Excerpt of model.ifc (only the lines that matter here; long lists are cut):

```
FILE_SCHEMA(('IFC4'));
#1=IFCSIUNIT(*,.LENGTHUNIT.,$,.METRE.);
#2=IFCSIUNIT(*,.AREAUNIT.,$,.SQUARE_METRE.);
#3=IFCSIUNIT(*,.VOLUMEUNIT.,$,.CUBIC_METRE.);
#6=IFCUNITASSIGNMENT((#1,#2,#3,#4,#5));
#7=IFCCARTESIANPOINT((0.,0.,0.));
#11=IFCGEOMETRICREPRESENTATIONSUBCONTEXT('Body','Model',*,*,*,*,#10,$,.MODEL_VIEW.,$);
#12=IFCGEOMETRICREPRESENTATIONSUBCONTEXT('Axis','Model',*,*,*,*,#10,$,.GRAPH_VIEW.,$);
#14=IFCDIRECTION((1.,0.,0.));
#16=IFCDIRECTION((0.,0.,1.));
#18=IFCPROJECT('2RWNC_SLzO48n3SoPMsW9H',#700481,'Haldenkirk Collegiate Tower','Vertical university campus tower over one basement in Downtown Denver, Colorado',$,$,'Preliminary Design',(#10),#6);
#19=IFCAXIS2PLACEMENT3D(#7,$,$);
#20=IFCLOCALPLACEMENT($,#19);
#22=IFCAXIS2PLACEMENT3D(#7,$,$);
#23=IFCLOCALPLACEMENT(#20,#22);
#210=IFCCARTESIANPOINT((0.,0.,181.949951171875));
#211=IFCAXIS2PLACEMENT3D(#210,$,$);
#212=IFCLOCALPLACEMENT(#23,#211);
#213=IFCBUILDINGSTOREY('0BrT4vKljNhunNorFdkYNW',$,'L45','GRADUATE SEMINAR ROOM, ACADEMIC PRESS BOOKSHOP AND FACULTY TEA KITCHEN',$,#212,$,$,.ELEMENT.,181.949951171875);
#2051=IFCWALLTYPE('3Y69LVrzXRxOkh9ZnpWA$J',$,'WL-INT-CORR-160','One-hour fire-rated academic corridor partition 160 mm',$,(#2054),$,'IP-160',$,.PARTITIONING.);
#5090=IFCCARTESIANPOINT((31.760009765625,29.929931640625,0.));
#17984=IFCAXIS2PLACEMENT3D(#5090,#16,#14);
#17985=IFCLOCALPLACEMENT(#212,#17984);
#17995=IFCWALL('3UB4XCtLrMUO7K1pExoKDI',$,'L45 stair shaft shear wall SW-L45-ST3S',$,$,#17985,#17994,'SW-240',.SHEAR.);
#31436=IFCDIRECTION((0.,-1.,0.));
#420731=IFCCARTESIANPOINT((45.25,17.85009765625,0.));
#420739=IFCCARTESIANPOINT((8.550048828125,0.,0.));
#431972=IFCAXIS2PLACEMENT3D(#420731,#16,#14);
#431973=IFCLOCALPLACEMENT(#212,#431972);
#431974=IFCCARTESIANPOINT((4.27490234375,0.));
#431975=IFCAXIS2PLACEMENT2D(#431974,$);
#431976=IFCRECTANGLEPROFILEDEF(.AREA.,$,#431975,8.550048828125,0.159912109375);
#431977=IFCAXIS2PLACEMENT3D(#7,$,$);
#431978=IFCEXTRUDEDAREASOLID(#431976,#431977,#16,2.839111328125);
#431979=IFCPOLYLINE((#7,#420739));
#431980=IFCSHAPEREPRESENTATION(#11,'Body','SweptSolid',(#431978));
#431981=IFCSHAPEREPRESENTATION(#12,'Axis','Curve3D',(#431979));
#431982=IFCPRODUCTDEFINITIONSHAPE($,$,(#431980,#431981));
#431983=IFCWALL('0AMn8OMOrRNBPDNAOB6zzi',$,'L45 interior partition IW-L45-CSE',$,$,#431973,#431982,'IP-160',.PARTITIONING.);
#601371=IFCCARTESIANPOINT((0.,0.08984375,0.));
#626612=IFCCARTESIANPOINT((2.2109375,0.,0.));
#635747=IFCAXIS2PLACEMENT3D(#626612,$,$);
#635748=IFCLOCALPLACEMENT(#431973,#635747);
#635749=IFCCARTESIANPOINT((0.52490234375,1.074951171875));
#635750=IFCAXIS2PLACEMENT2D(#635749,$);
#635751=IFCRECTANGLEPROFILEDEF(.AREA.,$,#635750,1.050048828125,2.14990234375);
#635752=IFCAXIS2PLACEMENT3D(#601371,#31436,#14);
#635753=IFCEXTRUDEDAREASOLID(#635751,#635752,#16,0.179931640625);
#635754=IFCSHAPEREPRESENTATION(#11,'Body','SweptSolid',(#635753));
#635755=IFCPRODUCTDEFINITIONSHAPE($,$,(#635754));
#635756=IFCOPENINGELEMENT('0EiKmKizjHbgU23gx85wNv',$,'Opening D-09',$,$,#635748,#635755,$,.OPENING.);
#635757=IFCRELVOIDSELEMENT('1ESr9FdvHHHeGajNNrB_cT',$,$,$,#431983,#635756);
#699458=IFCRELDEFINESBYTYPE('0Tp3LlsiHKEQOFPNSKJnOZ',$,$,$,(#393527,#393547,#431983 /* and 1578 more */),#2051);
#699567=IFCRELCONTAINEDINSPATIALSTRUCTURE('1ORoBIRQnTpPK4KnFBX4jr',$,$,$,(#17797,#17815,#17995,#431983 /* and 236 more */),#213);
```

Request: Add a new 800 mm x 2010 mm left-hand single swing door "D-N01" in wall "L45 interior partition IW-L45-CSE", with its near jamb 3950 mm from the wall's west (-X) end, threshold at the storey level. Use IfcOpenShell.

```python
import numpy as np
import ifcopenshell
import ifcopenshell.api.feature
import ifcopenshell.api.geometry
import ifcopenshell.api.root
import ifcopenshell.api.spatial
import ifcopenshell.geom
import ifcopenshell.util.element
import ifcopenshell.util.placement
import ifcopenshell.util.representation
import ifcopenshell.util.shape
import ifcopenshell.util.unit

model = ifcopenshell.open("model.ifc")
unit_scale = ifcopenshell.util.unit.calculate_unit_scale(model)
settings = ifcopenshell.geom.settings()


def volume(element):
    """Net volume in cubic metres, openings subtracted."""
    shape = ifcopenshell.geom.create_shape(settings, element)
    return ifcopenshell.util.shape.get_volume(shape.geometry)


wall = model.by_guid("0AMn8OMOrRNBPDNAOB6zzi")
storey = ifcopenshell.util.element.get_container(wall, ifc_class="IfcBuildingStorey")
context = ifcopenshell.util.representation.get_context(model, "Model", "Body", "MODEL_VIEW")
before = volume(wall)

width, height, from_end, sill = 0.8, 2.01, 3.95, 0.0  # metres

# The wall runs along its own X axis, and the end named is its -X end.
wall_shape = ifcopenshell.geom.create_shape(settings, wall)
x, y, z = ifcopenshell.util.shape.get_vertices(wall_shape.geometry).T
start = x.min() + from_end
face, thickness = float(y.min()), float(y.max() - y.min())
wall_matrix = ifcopenshell.util.placement.get_local_placement(wall.ObjectPlacement)
level = ifcopenshell.util.placement.get_local_placement(storey.ObjectPlacement)[2, 3]


def in_wall(x, y):
    """Placement at x, y metres in the wall's axes, at sill height."""
    matrix = wall_matrix.copy()
    matrix[:, 3] = wall_matrix @ np.array([x / unit_scale, y / unit_scale, 0.0, 1.0])
    matrix[2, 3] = level + sill / unit_scale
    return matrix


# Opening: a box that overshoots both wall faces by 50 mm.
opening = ifcopenshell.api.root.create_entity(model, ifc_class="IfcOpeningElement", predefined_type="OPENING")
box = ifcopenshell.api.geometry.add_wall_representation(
    model, context=context, length=width, height=height, thickness=thickness + 0.1
)
ifcopenshell.api.geometry.assign_representation(model, product=opening, representation=box)
ifcopenshell.api.geometry.edit_object_placement(model, product=opening, matrix=in_wall(start, face - 0.05), is_si=False)
ifcopenshell.api.feature.add_feature(model, feature=opening, element=wall)

door = ifcopenshell.api.root.create_entity(model, ifc_class="IfcDoor", name="D-N01", predefined_type="DOOR")
door.OverallWidth, door.OverallHeight = width / unit_scale, height / unit_scale
door.OperationType = "SINGLE_SWING_LEFT"
body = ifcopenshell.api.geometry.add_door_representation(
    model,
    context=context,
    overall_width=door.OverallWidth,
    overall_height=door.OverallHeight,
    operation_type="SINGLE_SWING_LEFT",
    lining_properties={"LiningDepth": thickness / unit_scale, "ThresholdDepth": thickness / unit_scale},
)
ifcopenshell.api.geometry.assign_representation(model, product=door, representation=body)
ifcopenshell.api.spatial.assign_container(model, products=[door], relating_structure=storey)
ifcopenshell.api.feature.add_filling(model, opening=opening, element=door)

# The lining spans the wall, so the door starts at the wall face.
ifcopenshell.api.geometry.edit_object_placement(model, product=door, matrix=in_wall(start, face), is_si=False)

after = volume(wall)

print(f"wall volume {before:.3f} -> {after:.3f} m3")

model.write("model_rev.ifc")
```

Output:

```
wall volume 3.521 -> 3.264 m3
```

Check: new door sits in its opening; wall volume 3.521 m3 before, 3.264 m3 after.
